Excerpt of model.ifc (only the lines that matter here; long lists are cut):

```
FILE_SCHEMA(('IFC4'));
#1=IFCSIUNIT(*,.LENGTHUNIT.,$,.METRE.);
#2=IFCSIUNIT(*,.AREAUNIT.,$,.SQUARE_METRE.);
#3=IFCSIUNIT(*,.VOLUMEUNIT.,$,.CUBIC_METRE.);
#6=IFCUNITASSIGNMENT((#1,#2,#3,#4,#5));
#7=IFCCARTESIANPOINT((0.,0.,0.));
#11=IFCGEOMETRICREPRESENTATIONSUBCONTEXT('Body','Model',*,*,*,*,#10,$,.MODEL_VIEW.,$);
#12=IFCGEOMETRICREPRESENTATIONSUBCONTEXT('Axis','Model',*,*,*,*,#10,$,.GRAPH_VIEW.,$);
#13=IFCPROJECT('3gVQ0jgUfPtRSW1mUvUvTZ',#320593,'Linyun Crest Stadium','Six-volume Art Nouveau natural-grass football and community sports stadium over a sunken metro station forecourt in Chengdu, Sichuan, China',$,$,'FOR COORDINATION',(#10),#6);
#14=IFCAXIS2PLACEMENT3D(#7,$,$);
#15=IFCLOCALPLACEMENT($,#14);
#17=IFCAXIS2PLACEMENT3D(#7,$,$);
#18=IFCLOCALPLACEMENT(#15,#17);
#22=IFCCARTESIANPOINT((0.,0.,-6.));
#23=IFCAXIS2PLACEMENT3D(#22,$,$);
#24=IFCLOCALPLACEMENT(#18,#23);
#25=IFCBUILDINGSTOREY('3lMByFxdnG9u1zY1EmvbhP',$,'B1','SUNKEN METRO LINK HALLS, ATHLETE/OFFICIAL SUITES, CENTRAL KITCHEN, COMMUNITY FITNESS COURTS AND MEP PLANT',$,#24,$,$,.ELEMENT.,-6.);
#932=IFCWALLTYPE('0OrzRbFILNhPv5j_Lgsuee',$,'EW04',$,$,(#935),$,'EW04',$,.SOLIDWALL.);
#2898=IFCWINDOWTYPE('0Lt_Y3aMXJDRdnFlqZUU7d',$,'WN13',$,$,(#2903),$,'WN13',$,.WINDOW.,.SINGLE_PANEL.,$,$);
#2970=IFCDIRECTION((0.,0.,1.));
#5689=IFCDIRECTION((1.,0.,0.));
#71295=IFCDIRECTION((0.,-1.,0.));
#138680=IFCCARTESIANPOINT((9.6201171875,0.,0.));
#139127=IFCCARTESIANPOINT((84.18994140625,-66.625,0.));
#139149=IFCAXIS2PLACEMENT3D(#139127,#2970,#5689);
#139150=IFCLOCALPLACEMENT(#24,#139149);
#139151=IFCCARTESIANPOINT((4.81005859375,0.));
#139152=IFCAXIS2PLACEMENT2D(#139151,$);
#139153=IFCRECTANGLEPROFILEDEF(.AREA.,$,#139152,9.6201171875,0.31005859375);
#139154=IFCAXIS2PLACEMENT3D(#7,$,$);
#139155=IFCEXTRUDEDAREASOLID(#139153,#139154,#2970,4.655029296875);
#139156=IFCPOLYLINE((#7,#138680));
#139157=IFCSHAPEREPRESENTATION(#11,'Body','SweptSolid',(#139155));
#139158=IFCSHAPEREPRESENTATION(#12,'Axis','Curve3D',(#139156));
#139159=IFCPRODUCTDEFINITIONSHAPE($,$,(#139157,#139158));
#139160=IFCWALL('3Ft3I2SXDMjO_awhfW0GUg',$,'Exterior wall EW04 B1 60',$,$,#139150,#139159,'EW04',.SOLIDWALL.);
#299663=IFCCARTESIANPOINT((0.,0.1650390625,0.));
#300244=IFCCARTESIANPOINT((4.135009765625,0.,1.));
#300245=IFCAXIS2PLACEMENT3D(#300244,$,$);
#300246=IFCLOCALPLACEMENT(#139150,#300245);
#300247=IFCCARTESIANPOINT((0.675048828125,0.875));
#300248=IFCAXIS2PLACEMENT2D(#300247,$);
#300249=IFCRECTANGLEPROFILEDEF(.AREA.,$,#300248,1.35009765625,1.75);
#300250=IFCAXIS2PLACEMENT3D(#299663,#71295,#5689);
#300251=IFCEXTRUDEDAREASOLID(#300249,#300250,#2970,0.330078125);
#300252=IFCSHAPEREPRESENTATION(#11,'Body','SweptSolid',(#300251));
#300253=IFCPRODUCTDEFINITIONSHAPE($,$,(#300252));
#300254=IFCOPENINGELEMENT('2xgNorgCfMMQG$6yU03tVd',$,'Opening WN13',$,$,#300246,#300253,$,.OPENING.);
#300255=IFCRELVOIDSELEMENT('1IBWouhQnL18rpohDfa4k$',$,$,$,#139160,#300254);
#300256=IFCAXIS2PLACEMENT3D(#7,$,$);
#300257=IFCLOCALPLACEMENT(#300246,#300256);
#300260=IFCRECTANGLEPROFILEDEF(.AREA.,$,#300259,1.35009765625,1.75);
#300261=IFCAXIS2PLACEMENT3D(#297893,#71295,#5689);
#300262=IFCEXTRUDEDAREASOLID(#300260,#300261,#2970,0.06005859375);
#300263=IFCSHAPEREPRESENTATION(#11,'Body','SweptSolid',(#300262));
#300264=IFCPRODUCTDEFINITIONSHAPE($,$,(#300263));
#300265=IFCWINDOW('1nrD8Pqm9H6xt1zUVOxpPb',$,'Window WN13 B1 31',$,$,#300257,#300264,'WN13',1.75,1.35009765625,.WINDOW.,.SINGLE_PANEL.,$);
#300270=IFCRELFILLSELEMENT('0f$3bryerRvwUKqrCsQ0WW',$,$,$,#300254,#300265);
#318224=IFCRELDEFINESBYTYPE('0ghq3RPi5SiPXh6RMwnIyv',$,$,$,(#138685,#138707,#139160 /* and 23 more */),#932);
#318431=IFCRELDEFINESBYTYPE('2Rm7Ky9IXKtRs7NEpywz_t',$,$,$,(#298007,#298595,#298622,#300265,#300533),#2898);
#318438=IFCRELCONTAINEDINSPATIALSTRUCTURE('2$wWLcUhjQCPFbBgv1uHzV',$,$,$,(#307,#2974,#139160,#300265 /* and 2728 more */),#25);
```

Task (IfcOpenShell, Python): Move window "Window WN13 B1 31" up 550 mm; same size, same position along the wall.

```python
import numpy as np
import ifcopenshell
import ifcopenshell.api.geometry
import ifcopenshell.util.placement
import ifcopenshell.util.unit

model = ifcopenshell.open("model.ifc")
unit_scale = ifcopenshell.util.unit.calculate_unit_scale(model)

window = model.by_guid("1nrD8Pqm9H6xt1zUVOxpPb")
opening = window.FillsVoids[0].RelatingOpeningElement
dz = 0.55 / unit_scale

shift = np.array([0.0, 0.0, dz])
# The window is placed relative to its opening, so it follows when the opening moves.
matrix = ifcopenshell.util.placement.get_local_placement(opening.ObjectPlacement)
matrix[:3, 3] += shift
ifcopenshell.api.geometry.edit_object_placement(
    model, product=opening, matrix=matrix, is_si=False, should_transform_children=True
)

print(f"moved by {dz * unit_scale:+.3f} m")

model.write("model_rev.ifc")
```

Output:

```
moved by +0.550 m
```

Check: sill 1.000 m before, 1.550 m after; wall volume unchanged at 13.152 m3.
